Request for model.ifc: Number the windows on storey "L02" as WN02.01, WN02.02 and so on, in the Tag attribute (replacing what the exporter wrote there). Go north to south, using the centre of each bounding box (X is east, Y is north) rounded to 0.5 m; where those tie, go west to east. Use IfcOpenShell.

First a look at what the model holds.

```python
import ifcopenshell
import ifcopenshell.util.element
import ifcopenshell.util.placement

model = ifcopenshell.open("model.ifc")
print(model.schema)
storey = next(s for s in model.by_type("IfcBuildingStorey") if s.Name == "L02")
windows = [e for e in ifcopenshell.util.element.get_decomposition(storey) if e.is_a("IfcWindow")]
for e in sorted(windows, key=lambda e: e.id()):
    origin = ifcopenshell.util.placement.get_local_placement(e.ObjectPlacement)[:3, 3]
    print(e.id(), e.Tag, e.Name, origin.round(2) + 0.0, sep=" | ")
```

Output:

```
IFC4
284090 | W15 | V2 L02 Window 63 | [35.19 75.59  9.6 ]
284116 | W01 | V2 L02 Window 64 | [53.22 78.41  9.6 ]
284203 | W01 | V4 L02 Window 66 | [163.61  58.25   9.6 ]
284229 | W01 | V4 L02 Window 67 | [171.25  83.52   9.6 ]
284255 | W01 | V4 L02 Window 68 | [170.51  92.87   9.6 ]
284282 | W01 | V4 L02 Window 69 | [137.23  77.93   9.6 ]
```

```python
import ifcopenshell
import ifcopenshell.geom
import ifcopenshell.util.element
import ifcopenshell.util.shape

model = ifcopenshell.open("model.ifc")
settings = ifcopenshell.geom.settings()
settings.set("use-world-coords", True)


def centre(element):
    shape = ifcopenshell.geom.create_shape(settings, element)
    return ifcopenshell.util.shape.get_bbox_centroid(shape.geometry)


storey = next(s for s in model.by_type("IfcBuildingStorey") if s.Name == "L02")
windows = [e for e in ifcopenshell.util.element.get_decomposition(storey) if e.is_a("IfcWindow")]

# Insertion points can sit at a corner or the storey origin, so sort by the geometry (in metres).
centres = {e: centre(e) for e in windows}
windows.sort(key=lambda e: (-round(centres[e][1] / 0.5), centres[e][0]))

for i, e in enumerate(windows, start=1):
    number = f"WN02.{i:02d}"
    e.Tag = number
    print(e.id(), number)

model.write("model_rev.ifc")
```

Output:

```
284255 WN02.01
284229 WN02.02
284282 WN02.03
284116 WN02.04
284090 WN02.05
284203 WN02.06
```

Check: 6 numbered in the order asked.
